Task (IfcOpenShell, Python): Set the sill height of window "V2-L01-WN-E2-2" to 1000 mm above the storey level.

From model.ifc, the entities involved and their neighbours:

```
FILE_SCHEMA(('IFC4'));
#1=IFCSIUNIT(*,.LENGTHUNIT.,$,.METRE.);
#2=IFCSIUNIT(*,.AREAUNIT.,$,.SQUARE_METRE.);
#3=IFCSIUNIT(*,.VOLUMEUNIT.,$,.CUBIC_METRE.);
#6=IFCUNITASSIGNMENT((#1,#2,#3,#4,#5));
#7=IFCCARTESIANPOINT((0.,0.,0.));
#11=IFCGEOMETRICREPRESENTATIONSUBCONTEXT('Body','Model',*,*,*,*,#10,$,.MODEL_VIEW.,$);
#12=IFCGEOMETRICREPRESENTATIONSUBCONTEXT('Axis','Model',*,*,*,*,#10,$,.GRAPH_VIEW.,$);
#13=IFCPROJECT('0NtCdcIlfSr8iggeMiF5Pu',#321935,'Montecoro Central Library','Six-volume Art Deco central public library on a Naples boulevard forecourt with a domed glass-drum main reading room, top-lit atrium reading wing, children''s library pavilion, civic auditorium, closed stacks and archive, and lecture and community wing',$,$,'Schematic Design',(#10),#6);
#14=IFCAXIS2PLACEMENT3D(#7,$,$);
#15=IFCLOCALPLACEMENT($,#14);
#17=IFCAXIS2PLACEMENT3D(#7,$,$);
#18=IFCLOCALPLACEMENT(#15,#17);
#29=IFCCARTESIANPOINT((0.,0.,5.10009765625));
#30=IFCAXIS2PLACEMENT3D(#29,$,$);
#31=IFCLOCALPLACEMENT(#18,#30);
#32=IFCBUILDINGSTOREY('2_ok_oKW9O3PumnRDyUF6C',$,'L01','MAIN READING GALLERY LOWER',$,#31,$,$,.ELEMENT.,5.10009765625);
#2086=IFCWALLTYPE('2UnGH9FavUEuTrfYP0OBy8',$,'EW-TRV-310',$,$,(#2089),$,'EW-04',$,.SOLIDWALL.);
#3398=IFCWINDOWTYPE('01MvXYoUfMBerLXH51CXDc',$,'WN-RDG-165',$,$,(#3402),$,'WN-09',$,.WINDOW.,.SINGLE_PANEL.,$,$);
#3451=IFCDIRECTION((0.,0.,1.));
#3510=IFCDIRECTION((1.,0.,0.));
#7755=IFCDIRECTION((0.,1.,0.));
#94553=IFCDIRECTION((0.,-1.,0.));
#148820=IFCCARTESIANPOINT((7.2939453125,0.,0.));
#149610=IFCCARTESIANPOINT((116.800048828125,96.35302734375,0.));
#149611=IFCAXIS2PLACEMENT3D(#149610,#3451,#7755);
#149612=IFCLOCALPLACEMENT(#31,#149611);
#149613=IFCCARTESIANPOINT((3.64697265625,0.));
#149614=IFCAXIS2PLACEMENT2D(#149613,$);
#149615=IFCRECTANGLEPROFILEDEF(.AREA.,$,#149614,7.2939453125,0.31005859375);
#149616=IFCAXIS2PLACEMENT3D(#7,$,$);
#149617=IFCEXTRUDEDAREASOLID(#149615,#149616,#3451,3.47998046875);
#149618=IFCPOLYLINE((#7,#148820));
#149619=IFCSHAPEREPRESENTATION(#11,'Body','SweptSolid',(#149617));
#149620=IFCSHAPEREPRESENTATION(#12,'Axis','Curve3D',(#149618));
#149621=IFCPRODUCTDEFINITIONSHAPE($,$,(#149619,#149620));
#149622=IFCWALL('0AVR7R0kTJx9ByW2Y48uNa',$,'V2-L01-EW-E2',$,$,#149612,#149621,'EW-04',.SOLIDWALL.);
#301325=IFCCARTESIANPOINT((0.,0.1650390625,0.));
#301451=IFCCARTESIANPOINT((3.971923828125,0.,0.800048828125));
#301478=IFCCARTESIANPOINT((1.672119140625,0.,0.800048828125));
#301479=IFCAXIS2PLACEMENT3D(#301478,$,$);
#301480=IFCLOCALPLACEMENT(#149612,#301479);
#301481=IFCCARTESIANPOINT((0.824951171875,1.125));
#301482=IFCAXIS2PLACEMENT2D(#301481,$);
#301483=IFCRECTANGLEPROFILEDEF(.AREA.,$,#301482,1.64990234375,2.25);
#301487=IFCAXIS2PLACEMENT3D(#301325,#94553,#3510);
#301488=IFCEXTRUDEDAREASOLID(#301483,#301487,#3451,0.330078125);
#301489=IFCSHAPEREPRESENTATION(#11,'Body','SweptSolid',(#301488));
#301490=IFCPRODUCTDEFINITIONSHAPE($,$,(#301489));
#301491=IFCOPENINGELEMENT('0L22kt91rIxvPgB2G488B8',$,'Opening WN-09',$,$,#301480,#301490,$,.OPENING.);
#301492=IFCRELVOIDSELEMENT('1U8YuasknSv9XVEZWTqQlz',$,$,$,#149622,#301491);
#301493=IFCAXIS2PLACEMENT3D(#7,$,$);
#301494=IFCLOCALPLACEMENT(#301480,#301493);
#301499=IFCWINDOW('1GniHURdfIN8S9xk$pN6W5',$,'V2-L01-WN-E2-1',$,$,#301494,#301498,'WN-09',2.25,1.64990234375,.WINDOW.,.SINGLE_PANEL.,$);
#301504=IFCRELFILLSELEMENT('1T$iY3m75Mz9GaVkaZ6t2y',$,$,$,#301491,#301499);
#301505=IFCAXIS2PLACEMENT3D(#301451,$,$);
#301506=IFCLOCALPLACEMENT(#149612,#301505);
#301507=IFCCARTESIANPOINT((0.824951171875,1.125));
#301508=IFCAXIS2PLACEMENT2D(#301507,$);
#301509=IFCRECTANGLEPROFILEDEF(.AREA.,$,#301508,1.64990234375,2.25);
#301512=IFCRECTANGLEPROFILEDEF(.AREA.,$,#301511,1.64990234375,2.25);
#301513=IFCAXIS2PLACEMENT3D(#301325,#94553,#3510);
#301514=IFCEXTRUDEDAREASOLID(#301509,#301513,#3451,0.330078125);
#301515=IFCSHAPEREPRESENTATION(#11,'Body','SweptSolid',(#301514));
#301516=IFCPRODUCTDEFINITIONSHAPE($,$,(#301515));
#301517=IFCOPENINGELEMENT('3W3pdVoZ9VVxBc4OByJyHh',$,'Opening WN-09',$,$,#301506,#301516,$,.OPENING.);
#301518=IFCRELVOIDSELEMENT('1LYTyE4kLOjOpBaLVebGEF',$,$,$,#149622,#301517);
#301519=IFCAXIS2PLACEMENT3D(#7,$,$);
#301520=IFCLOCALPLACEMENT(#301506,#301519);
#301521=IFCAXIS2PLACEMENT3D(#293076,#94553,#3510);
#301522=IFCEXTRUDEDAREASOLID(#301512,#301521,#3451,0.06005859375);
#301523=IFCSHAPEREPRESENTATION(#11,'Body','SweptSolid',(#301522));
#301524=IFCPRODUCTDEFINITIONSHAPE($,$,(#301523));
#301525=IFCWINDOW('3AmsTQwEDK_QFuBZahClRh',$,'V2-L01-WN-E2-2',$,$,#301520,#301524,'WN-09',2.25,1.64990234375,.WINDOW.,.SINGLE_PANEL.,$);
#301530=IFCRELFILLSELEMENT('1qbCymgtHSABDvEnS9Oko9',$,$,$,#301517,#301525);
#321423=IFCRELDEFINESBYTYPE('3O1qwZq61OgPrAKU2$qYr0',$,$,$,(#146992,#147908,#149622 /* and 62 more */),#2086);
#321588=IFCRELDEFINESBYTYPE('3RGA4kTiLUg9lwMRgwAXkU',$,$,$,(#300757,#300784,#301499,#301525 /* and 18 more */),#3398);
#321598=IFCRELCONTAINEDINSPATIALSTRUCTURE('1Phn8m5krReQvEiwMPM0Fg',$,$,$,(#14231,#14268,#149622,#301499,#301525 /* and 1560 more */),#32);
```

```python
import numpy as np
import ifcopenshell
import ifcopenshell.api.geometry
import ifcopenshell.geom
import ifcopenshell.util.element
import ifcopenshell.util.placement
import ifcopenshell.util.shape
import ifcopenshell.util.unit

model = ifcopenshell.open("model.ifc")
unit_scale = ifcopenshell.util.unit.calculate_unit_scale(model)

window = model.by_id(301525)
opening = window.FillsVoids[0].RelatingOpeningElement
storey = ifcopenshell.util.element.get_container(window, ifc_class="IfcBuildingStorey")
level = ifcopenshell.util.placement.get_local_placement(storey.ObjectPlacement)[2, 3]

# The opening's origin need not be at the sill, so measure its lowest point.
shape = ifcopenshell.geom.create_shape(ifcopenshell.geom.settings(), opening)
bottom = ifcopenshell.util.shape.get_shape_bottom_elevation(shape, shape.geometry) / unit_scale
dz = level + 1 / unit_scale - bottom

shift = np.array([0.0, 0.0, dz])
# The window is placed relative to its opening, so it follows when the opening moves.
matrix = ifcopenshell.util.placement.get_local_placement(opening.ObjectPlacement)
matrix[:3, 3] += shift
ifcopenshell.api.geometry.edit_object_placement(
    model, product=opening, matrix=matrix, is_si=False, should_transform_children=True
)

print(f"moved by {dz * unit_scale:+.3f} m")

model.write("model-out.ifc")
```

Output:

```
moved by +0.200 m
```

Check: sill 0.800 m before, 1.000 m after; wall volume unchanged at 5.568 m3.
